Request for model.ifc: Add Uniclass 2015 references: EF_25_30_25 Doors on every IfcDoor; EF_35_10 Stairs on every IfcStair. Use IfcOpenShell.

First a look at what the model holds.

```python
import ifcopenshell

model = ifcopenshell.open("model.ifc")
print(model.schema)
print("classifications:", [c.Name for c in model.by_type("IfcClassification")])
for ifc_class in ("IfcDoor", "IfcRoof", "IfcStair", "IfcWall", "IfcWindow"):
    print(ifc_class, len(model.by_type(ifc_class)))
```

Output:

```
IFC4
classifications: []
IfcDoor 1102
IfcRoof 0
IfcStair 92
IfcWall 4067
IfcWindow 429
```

```python
import ifcopenshell
import ifcopenshell.api.classification

model = ifcopenshell.open("model.ifc")

system = ifcopenshell.api.classification.add_classification(model, classification="Uniclass 2015")

codes = {
    "IfcDoor": ("EF_25_30_25", "Doors"),
    "IfcStair": ("EF_35_10", "Stairs"),
}
for ifc_class, (code, name) in codes.items():
    products = model.by_type(ifc_class)
    ifcopenshell.api.classification.add_reference(
        model, products=products, classification=system, identification=code, name=name
    )
    print(code, len(products))

model.write("model_edited.ifc")
```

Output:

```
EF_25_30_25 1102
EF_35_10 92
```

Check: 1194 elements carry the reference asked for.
